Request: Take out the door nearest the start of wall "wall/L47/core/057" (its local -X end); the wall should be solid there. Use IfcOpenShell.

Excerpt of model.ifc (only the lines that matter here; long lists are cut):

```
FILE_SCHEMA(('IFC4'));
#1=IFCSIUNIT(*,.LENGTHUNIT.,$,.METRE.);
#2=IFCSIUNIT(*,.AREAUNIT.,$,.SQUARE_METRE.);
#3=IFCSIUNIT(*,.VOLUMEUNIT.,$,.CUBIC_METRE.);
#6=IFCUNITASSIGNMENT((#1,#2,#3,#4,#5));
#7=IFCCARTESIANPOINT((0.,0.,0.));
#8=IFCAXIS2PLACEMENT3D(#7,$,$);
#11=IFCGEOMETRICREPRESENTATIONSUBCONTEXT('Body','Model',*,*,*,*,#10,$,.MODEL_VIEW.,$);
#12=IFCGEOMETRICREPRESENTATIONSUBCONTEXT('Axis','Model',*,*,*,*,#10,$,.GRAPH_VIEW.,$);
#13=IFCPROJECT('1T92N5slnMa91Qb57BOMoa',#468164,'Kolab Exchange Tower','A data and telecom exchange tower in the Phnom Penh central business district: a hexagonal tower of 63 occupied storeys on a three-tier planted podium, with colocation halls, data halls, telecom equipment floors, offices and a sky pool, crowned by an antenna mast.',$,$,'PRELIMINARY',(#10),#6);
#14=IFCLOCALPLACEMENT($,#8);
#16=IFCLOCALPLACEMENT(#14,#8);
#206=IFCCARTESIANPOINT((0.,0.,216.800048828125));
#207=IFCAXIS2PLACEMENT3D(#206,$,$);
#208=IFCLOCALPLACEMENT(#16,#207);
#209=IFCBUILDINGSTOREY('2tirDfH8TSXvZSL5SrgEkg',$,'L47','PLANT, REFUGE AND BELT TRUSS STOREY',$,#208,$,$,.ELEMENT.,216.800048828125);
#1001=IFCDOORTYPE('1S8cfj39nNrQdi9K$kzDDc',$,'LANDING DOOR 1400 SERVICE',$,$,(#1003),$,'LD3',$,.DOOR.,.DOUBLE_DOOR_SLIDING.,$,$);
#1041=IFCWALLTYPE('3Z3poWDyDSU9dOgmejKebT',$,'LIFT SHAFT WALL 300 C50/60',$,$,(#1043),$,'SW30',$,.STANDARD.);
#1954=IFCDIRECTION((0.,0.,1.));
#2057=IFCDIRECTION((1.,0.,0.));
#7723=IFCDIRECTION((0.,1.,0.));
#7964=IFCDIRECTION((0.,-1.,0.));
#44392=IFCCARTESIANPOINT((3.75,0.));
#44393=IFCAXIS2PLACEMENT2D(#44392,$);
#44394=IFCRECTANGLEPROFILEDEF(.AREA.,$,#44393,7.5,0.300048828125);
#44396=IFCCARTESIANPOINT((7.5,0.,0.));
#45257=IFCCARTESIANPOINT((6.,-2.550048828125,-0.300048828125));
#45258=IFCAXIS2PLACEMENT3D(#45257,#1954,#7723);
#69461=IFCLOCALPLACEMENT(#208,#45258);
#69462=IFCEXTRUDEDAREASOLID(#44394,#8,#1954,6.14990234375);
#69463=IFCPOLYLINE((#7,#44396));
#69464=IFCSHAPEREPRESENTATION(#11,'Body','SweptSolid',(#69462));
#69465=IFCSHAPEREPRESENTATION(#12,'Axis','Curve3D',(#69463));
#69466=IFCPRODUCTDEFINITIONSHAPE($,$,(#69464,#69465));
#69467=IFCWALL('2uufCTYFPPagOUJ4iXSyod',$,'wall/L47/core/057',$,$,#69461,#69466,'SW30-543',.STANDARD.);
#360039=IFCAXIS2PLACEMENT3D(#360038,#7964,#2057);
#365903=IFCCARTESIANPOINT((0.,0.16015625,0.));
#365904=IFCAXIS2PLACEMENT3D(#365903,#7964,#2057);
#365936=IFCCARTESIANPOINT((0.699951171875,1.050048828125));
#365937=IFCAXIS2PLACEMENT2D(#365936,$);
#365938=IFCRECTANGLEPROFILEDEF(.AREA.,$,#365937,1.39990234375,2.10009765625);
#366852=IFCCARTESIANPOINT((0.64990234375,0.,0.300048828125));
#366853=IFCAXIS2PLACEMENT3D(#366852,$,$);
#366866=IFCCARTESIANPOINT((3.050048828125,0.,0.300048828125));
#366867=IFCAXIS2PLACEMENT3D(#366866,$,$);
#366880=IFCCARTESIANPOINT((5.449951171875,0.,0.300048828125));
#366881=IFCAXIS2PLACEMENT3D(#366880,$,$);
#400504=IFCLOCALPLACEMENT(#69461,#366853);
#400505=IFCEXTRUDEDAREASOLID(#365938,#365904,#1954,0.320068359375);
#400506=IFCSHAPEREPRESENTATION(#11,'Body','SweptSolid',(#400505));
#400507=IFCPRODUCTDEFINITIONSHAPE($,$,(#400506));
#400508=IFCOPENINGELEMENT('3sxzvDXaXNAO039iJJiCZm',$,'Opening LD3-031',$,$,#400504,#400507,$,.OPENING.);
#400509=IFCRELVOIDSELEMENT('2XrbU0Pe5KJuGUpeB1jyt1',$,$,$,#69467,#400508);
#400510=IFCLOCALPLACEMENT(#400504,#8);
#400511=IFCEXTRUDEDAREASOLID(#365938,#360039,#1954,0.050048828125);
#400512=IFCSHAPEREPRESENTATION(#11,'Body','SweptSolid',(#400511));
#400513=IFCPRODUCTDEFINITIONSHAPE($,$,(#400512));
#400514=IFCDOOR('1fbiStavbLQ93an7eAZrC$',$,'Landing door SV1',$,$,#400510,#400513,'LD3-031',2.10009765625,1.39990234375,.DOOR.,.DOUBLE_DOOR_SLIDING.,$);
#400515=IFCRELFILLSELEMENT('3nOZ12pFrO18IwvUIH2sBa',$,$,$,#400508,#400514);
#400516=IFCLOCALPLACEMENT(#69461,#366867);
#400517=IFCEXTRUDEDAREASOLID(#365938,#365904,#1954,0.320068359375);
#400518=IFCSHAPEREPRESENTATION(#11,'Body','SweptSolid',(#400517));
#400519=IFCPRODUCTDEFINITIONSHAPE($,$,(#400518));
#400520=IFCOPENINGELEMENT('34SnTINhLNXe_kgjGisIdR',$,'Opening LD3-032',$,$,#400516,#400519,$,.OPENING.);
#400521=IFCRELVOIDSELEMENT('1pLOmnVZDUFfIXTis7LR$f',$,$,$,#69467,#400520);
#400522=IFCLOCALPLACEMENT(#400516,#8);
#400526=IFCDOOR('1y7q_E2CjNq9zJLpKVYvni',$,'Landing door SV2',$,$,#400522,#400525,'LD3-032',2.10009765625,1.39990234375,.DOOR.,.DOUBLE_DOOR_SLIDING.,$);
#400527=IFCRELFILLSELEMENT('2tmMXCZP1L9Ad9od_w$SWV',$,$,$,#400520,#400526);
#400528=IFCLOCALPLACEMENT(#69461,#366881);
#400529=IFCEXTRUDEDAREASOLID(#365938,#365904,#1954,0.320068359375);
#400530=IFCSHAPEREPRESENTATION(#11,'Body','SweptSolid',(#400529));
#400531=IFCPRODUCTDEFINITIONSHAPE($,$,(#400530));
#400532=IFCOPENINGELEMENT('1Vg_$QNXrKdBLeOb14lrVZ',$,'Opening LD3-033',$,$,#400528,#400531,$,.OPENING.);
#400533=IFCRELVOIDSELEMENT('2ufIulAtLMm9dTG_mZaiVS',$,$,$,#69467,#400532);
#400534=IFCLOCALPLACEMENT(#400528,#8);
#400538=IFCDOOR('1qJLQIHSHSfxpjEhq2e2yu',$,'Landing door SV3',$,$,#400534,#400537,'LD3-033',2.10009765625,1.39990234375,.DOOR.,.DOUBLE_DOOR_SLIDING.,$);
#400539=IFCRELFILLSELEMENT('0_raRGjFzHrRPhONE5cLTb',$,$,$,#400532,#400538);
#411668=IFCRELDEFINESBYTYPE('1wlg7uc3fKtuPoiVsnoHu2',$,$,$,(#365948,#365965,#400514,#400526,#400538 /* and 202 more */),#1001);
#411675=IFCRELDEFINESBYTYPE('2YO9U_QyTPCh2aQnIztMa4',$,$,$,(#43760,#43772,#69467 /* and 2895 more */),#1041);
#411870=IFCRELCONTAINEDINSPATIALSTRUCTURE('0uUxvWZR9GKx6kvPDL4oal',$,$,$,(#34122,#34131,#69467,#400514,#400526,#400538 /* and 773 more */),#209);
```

```python
import ifcopenshell
import ifcopenshell.api.feature
import ifcopenshell.api.root
import ifcopenshell.geom
import ifcopenshell.util.shape

model = ifcopenshell.open("model.ifc")
settings = ifcopenshell.geom.settings()


def volume(element):
    """Net volume in cubic metres, openings subtracted."""
    shape = ifcopenshell.geom.create_shape(settings, element)
    return ifcopenshell.util.shape.get_volume(shape.geometry)


door = model.by_guid("1fbiStavbLQ93an7eAZrC$")
opening = door.FillsVoids[0].RelatingOpeningElement
wall = opening.VoidsElements[0].RelatingBuildingElement
before = volume(wall)

ifcopenshell.api.root.remove_product(model, product=door)
ifcopenshell.api.feature.remove_feature(model, feature=opening)

after = volume(wall)

print(f"wall volume {before:.3f} -> {after:.3f} m3")

model.write("model_updated.ifc")
```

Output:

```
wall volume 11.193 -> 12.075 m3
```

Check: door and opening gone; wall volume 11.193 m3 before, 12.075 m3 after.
